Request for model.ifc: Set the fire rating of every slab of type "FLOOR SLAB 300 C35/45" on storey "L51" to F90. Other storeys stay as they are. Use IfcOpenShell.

First a look at what the model holds.

```python
import ifcopenshell
import ifcopenshell.util.element

model = ifcopenshell.open("model.ifc")
print(model.schema)
storey = next(s for s in model.by_type("IfcBuildingStorey") if s.Name == "L51")
slabs = [e for e in ifcopenshell.util.element.get_decomposition(storey) if e.is_a("IfcSlab")]
seen = {}
for e in slabs:
    element_type = ifcopenshell.util.element.get_type(e)
    key = (element_type.Name if element_type != e and element_type else None, ifcopenshell.util.element.get_pset(e, "Pset_SlabCommon", "FireRating"))
    seen[key] = seen.get(key, 0) + 1
for (name, value), count in sorted(seen.items(), key=str):
    print(count, "x", name, "|", value)
```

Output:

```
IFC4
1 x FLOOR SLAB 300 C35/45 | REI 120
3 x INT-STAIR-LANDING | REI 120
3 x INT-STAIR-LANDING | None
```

```python
import ifcopenshell
import ifcopenshell.api.pset
import ifcopenshell.util.element

model = ifcopenshell.open("model.ifc")

storey = next(s for s in model.by_type("IfcBuildingStorey") if s.Name == "L51")
slabs = [e for e in ifcopenshell.util.element.get_decomposition(storey) if e.is_a("IfcSlab")]

count = 0
for e in slabs:
    element_type = ifcopenshell.util.element.get_type(e)
    if element_type in (None, e) or element_type.Name != "FLOOR SLAB 300 C35/45":
        continue
    found = ifcopenshell.util.element.get_pset(e, "Pset_SlabCommon", should_inherit=False)
    if found:
        pset = model.by_id(found["id"])
        if len(ifcopenshell.util.element.get_elements_by_pset(pset)) > 1:
            pset = ifcopenshell.api.pset.unshare_pset(model, products=[e], pset=pset)[0]
    else:
        pset = ifcopenshell.api.pset.add_pset(model, product=e, name="Pset_SlabCommon")
    ifcopenshell.api.pset.edit_pset(model, pset=pset, properties={"FireRating": "F90"})
    count += 1

print(count, "slabs updated")

model.write("model_updated.ifc")
```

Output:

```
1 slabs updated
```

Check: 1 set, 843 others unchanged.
